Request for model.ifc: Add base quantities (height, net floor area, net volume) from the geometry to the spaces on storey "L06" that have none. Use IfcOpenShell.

First a look at what the model holds.

```python
import ifcopenshell
import ifcopenshell.util.element
import ifcopenshell.util.unit

model = ifcopenshell.open("model.ifc")
print(model.schema)
for unit_type in ("LENGTHUNIT", "AREAUNIT", "VOLUMEUNIT"):
    print(unit_type, ifcopenshell.util.unit.calculate_unit_scale(model, unit_type))
storey = next(s for s in model.by_type("IfcBuildingStorey") if s.Name == "L06")
spaces = [e for e in ifcopenshell.util.element.get_decomposition(storey) if e.is_a("IfcSpace")]
for e in sorted(spaces, key=lambda e: e.id()):
    print(e.id(), e.is_a(), e.Name, list(ifcopenshell.util.element.get_psets(e, qtos_only=True)), sep=" | ")
```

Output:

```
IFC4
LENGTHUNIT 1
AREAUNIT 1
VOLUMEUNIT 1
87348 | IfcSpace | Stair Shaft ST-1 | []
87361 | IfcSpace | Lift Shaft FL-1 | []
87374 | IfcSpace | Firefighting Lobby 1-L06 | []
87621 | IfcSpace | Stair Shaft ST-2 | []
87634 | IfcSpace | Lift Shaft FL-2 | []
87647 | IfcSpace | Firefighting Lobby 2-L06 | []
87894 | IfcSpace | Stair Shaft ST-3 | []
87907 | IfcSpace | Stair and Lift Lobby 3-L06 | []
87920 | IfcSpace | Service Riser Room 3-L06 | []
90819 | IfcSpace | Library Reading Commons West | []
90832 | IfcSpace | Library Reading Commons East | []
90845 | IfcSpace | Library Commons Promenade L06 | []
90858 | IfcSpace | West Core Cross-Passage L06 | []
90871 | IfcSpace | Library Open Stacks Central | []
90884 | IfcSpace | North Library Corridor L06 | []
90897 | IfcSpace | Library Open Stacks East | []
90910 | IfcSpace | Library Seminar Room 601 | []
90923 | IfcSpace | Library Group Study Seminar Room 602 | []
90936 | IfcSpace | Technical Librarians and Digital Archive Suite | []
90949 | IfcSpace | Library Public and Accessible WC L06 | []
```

```python
import ifcopenshell
import ifcopenshell.api.pset
import ifcopenshell.geom
import ifcopenshell.util.element
import ifcopenshell.util.shape
import ifcopenshell.util.unit

model = ifcopenshell.open("model.ifc")
unit_scale = ifcopenshell.util.unit.calculate_unit_scale(model)
area_scale = ifcopenshell.util.unit.calculate_unit_scale(model, "AREAUNIT")
volume_scale = ifcopenshell.util.unit.calculate_unit_scale(model, "VOLUMEUNIT")
settings = ifcopenshell.geom.settings()

storey = next(s for s in model.by_type("IfcBuildingStorey") if s.Name == "L06")
spaces = [e for e in ifcopenshell.util.element.get_decomposition(storey) if e.is_a("IfcSpace")]

for e in sorted(spaces, key=lambda e: e.id()):
    if ifcopenshell.util.element.get_psets(e, qtos_only=True, should_inherit=False):
        continue
    # Geometry comes back in metres, in the element's own axes.
    shape = ifcopenshell.geom.create_shape(settings, e)
    values = {
        "Height": ifcopenshell.util.shape.get_z(shape.geometry) / unit_scale,
        "NetFloorArea": ifcopenshell.util.shape.get_footprint_area(shape.geometry) / area_scale,
        "NetVolume": ifcopenshell.util.shape.get_volume(shape.geometry) / volume_scale,
    }
    qto = ifcopenshell.api.pset.add_qto(model, product=e, name="Qto_SpaceBaseQuantities")
    ifcopenshell.api.pset.edit_qto(model, qto=qto, properties=values)
    print(e.id(), {k: round(v, 3) for k, v in values.items()})

model.write("model_rev.ifc")
```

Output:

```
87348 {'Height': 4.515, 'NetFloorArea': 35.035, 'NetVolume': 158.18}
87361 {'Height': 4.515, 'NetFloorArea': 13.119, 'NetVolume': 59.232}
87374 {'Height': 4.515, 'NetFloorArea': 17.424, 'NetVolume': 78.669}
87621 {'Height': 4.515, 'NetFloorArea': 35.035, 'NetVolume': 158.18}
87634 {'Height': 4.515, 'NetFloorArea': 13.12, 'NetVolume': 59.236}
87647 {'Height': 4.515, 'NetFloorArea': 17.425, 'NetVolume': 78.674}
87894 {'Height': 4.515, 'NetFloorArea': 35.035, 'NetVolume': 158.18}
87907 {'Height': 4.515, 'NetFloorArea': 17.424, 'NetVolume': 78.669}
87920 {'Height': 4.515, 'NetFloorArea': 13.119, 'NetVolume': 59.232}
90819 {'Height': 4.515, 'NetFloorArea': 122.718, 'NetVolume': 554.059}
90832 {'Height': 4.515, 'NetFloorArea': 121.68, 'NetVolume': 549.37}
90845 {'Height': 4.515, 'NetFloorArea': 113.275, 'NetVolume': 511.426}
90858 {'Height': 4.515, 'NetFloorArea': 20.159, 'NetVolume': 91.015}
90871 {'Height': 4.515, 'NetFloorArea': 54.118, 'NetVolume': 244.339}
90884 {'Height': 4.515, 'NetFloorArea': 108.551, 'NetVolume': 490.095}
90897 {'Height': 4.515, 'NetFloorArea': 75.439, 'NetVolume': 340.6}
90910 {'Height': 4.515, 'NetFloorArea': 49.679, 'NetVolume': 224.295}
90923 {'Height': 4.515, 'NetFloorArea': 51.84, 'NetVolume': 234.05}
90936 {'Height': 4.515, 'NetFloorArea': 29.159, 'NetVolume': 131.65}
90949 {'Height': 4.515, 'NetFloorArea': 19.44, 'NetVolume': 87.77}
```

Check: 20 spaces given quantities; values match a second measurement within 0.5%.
